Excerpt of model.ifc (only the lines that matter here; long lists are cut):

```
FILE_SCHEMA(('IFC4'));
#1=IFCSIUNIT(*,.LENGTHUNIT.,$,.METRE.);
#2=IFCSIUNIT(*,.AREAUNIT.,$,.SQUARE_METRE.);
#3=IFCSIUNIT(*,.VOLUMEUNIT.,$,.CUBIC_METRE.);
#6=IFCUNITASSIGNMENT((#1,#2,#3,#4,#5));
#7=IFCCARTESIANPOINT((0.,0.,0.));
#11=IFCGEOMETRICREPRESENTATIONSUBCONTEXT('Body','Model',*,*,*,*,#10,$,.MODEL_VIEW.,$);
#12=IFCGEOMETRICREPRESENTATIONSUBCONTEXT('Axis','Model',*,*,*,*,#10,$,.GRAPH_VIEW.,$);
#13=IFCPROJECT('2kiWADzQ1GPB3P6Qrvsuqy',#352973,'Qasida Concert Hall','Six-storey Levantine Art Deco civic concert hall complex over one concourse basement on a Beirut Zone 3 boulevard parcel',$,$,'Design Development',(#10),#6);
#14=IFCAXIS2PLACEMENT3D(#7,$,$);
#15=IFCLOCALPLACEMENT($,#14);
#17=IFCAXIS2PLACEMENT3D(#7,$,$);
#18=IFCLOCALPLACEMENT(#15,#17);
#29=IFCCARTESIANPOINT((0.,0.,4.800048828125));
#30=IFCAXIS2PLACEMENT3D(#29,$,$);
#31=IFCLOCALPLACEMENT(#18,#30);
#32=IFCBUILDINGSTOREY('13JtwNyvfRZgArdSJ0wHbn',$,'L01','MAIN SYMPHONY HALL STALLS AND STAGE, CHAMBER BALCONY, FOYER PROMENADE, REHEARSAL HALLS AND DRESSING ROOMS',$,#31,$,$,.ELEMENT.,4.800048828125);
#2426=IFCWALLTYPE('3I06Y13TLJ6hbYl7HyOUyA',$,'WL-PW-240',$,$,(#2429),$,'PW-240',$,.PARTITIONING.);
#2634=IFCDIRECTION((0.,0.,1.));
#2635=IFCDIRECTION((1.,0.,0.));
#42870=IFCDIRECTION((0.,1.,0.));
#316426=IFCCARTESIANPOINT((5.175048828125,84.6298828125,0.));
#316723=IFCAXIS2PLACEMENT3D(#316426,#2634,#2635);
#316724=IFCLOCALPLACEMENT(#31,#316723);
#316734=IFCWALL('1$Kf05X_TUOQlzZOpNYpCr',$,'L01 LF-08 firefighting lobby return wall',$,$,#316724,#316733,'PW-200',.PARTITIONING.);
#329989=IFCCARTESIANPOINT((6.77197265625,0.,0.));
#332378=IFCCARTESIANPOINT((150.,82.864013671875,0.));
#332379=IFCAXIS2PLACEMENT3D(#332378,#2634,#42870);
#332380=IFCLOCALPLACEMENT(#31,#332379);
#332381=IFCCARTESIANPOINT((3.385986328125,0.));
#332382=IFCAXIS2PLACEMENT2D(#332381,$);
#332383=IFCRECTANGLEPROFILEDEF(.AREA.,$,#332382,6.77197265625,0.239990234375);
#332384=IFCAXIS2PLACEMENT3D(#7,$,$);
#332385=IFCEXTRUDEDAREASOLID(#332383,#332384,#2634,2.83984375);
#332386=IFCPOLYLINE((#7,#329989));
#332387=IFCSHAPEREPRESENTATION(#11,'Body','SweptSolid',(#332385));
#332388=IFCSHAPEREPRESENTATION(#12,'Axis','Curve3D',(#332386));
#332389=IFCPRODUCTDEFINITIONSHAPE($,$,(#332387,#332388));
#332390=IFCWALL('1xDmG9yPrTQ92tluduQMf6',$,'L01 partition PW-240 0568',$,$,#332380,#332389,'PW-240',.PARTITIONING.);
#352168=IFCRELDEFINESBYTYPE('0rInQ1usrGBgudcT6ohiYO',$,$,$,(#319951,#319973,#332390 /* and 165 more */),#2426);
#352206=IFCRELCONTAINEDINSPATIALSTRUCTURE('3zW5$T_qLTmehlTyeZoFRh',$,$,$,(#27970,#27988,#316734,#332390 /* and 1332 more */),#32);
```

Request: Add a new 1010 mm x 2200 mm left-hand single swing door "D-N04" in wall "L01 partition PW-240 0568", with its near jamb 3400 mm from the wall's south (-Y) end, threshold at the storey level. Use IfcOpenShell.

```python
import numpy as np
import ifcopenshell
import ifcopenshell.api.feature
import ifcopenshell.api.geometry
import ifcopenshell.api.root
import ifcopenshell.api.spatial
import ifcopenshell.geom
import ifcopenshell.util.element
import ifcopenshell.util.placement
import ifcopenshell.util.representation
import ifcopenshell.util.shape
import ifcopenshell.util.unit

model = ifcopenshell.open("model.ifc")
unit_scale = ifcopenshell.util.unit.calculate_unit_scale(model)
settings = ifcopenshell.geom.settings()


def volume(element):
    """Net volume in cubic metres, openings subtracted."""
    shape = ifcopenshell.geom.create_shape(settings, element)
    return ifcopenshell.util.shape.get_volume(shape.geometry)


wall = model.by_id(332390)
storey = ifcopenshell.util.element.get_container(wall, ifc_class="IfcBuildingStorey")
context = ifcopenshell.util.representation.get_context(model, "Model", "Body", "MODEL_VIEW")
before = volume(wall)

width, height, from_end, sill = 1.01, 2.2, 3.4, 0.0  # metres

# The wall runs along its own X axis, and the end named is its -X end.
wall_shape = ifcopenshell.geom.create_shape(settings, wall)
x, y, z = ifcopenshell.util.shape.get_vertices(wall_shape.geometry).T
start = x.min() + from_end
face, thickness = float(y.min()), float(y.max() - y.min())
wall_matrix = ifcopenshell.util.placement.get_local_placement(wall.ObjectPlacement)
level = ifcopenshell.util.placement.get_local_placement(storey.ObjectPlacement)[2, 3]


def in_wall(x, y):
    """Placement at x, y metres in the wall's axes, at sill height."""
    matrix = wall_matrix.copy()
    matrix[:, 3] = wall_matrix @ np.array([x / unit_scale, y / unit_scale, 0.0, 1.0])
    matrix[2, 3] = level + sill / unit_scale
    return matrix


# Opening: a box that overshoots both wall faces by 50 mm.
opening = ifcopenshell.api.root.create_entity(model, ifc_class="IfcOpeningElement", predefined_type="OPENING")
box = ifcopenshell.api.geometry.add_wall_representation(
    model, context=context, length=width, height=height, thickness=thickness + 0.1
)
ifcopenshell.api.geometry.assign_representation(model, product=opening, representation=box)
ifcopenshell.api.geometry.edit_object_placement(model, product=opening, matrix=in_wall(start, face - 0.05), is_si=False)
ifcopenshell.api.feature.add_feature(model, feature=opening, element=wall)

door = ifcopenshell.api.root.create_entity(model, ifc_class="IfcDoor", name="D-N04", predefined_type="DOOR")
door.OverallWidth, door.OverallHeight = width / unit_scale, height / unit_scale
door.OperationType = "SINGLE_SWING_LEFT"
body = ifcopenshell.api.geometry.add_door_representation(
    model,
    context=context,
    overall_width=door.OverallWidth,
    overall_height=door.OverallHeight,
    operation_type="SINGLE_SWING_LEFT",
    lining_properties={"LiningDepth": thickness / unit_scale, "ThresholdDepth": thickness / unit_scale},
)
ifcopenshell.api.geometry.assign_representation(model, product=door, representation=body)
ifcopenshell.api.spatial.assign_container(model, products=[door], relating_structure=storey)
ifcopenshell.api.feature.add_filling(model, opening=opening, element=door)

# The lining spans the wall, so the door starts at the wall face.
ifcopenshell.api.geometry.edit_object_placement(model, product=door, matrix=in_wall(start, face), is_si=False)

after = volume(wall)

print(f"wall volume {before:.3f} -> {after:.3f} m3")

model.write("model-out.ifc")
```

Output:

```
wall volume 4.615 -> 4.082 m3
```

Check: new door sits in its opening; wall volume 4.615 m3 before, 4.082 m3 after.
